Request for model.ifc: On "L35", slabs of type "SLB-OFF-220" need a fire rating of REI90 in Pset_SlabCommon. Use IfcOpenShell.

First a look at what the model holds.

```python
import ifcopenshell
import ifcopenshell.util.element

model = ifcopenshell.open("model.ifc")
print(model.schema)
storey = next(s for s in model.by_type("IfcBuildingStorey") if s.Name == "L35")
slabs = [e for e in ifcopenshell.util.element.get_decomposition(storey) if e.is_a("IfcSlab")]
seen = {}
for e in slabs:
    element_type = ifcopenshell.util.element.get_type(e)
    key = (element_type.Name if element_type != e and element_type else None, ifcopenshell.util.element.get_pset(e, "Pset_SlabCommon", "FireRating"))
    seen[key] = seen.get(key, 0) + 1
for (name, value), count in sorted(seen.items(), key=str):
    print(count, "x", name, "|", value)
```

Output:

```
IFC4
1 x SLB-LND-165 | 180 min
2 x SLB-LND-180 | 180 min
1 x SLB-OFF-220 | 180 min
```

```python
import ifcopenshell
import ifcopenshell.api.pset
import ifcopenshell.util.element

model = ifcopenshell.open("model.ifc")

storey = next(s for s in model.by_type("IfcBuildingStorey") if s.Name == "L35")
slabs = [e for e in ifcopenshell.util.element.get_decomposition(storey) if e.is_a("IfcSlab")]

count = 0
for e in slabs:
    element_type = ifcopenshell.util.element.get_type(e)
    if element_type in (None, e) or element_type.Name != "SLB-OFF-220":
        continue
    found = ifcopenshell.util.element.get_pset(e, "Pset_SlabCommon", should_inherit=False)
    if found:
        pset = model.by_id(found["id"])
        if len(ifcopenshell.util.element.get_elements_by_pset(pset)) > 1:
            pset = ifcopenshell.api.pset.unshare_pset(model, products=[e], pset=pset)[0]
    else:
        pset = ifcopenshell.api.pset.add_pset(model, product=e, name="Pset_SlabCommon")
    ifcopenshell.api.pset.edit_pset(model, pset=pset, properties={"FireRating": "REI90"})
    count += 1

print(count, "slabs updated")

model.write("model_edited.ifc")
```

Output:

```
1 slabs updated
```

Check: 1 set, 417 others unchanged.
